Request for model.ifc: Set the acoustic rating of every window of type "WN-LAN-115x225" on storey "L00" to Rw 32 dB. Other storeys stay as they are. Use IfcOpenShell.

First a look at what the model holds.

```python
import ifcopenshell
import ifcopenshell.util.element

model = ifcopenshell.open("model.ifc")
print(model.schema)
storey = next(s for s in model.by_type("IfcBuildingStorey") if s.Name == "L00")
windows = [e for e in ifcopenshell.util.element.get_decomposition(storey) if e.is_a("IfcWindow")]
seen = {}
for e in windows:
    element_type = ifcopenshell.util.element.get_type(e)
    key = (element_type.Name if element_type != e and element_type else None, ifcopenshell.util.element.get_pset(e, "Pset_WindowCommon", "AcousticRating"))
    seen[key] = seen.get(key, 0) + 1
for (name, value), count in sorted(seen.items(), key=str):
    print(count, "x", name, "|", value)
```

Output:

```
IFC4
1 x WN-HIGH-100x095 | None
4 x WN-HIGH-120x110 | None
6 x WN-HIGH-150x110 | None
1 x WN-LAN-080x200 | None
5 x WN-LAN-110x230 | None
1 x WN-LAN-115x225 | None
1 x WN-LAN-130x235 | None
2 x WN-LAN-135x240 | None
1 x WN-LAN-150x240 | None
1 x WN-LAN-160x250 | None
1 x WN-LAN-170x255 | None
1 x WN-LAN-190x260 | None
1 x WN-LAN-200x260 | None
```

```python
import ifcopenshell
import ifcopenshell.api.pset
import ifcopenshell.util.element

model = ifcopenshell.open("model.ifc")

storey = next(s for s in model.by_type("IfcBuildingStorey") if s.Name == "L00")
windows = [e for e in ifcopenshell.util.element.get_decomposition(storey) if e.is_a("IfcWindow")]

count = 0
for e in windows:
    element_type = ifcopenshell.util.element.get_type(e)
    if element_type in (None, e) or element_type.Name != "WN-LAN-115x225":
        continue
    # add_pset returns the element's existing set when there is one.
    pset = ifcopenshell.api.pset.add_pset(model, product=e, name="Pset_WindowCommon")
    ifcopenshell.api.pset.edit_pset(model, pset=pset, properties={"AcousticRating": "Rw 32 dB"})
    count += 1

print(count, "windows updated")

model.write("model_edited.ifc")
```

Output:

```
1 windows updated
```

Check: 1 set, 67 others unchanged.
